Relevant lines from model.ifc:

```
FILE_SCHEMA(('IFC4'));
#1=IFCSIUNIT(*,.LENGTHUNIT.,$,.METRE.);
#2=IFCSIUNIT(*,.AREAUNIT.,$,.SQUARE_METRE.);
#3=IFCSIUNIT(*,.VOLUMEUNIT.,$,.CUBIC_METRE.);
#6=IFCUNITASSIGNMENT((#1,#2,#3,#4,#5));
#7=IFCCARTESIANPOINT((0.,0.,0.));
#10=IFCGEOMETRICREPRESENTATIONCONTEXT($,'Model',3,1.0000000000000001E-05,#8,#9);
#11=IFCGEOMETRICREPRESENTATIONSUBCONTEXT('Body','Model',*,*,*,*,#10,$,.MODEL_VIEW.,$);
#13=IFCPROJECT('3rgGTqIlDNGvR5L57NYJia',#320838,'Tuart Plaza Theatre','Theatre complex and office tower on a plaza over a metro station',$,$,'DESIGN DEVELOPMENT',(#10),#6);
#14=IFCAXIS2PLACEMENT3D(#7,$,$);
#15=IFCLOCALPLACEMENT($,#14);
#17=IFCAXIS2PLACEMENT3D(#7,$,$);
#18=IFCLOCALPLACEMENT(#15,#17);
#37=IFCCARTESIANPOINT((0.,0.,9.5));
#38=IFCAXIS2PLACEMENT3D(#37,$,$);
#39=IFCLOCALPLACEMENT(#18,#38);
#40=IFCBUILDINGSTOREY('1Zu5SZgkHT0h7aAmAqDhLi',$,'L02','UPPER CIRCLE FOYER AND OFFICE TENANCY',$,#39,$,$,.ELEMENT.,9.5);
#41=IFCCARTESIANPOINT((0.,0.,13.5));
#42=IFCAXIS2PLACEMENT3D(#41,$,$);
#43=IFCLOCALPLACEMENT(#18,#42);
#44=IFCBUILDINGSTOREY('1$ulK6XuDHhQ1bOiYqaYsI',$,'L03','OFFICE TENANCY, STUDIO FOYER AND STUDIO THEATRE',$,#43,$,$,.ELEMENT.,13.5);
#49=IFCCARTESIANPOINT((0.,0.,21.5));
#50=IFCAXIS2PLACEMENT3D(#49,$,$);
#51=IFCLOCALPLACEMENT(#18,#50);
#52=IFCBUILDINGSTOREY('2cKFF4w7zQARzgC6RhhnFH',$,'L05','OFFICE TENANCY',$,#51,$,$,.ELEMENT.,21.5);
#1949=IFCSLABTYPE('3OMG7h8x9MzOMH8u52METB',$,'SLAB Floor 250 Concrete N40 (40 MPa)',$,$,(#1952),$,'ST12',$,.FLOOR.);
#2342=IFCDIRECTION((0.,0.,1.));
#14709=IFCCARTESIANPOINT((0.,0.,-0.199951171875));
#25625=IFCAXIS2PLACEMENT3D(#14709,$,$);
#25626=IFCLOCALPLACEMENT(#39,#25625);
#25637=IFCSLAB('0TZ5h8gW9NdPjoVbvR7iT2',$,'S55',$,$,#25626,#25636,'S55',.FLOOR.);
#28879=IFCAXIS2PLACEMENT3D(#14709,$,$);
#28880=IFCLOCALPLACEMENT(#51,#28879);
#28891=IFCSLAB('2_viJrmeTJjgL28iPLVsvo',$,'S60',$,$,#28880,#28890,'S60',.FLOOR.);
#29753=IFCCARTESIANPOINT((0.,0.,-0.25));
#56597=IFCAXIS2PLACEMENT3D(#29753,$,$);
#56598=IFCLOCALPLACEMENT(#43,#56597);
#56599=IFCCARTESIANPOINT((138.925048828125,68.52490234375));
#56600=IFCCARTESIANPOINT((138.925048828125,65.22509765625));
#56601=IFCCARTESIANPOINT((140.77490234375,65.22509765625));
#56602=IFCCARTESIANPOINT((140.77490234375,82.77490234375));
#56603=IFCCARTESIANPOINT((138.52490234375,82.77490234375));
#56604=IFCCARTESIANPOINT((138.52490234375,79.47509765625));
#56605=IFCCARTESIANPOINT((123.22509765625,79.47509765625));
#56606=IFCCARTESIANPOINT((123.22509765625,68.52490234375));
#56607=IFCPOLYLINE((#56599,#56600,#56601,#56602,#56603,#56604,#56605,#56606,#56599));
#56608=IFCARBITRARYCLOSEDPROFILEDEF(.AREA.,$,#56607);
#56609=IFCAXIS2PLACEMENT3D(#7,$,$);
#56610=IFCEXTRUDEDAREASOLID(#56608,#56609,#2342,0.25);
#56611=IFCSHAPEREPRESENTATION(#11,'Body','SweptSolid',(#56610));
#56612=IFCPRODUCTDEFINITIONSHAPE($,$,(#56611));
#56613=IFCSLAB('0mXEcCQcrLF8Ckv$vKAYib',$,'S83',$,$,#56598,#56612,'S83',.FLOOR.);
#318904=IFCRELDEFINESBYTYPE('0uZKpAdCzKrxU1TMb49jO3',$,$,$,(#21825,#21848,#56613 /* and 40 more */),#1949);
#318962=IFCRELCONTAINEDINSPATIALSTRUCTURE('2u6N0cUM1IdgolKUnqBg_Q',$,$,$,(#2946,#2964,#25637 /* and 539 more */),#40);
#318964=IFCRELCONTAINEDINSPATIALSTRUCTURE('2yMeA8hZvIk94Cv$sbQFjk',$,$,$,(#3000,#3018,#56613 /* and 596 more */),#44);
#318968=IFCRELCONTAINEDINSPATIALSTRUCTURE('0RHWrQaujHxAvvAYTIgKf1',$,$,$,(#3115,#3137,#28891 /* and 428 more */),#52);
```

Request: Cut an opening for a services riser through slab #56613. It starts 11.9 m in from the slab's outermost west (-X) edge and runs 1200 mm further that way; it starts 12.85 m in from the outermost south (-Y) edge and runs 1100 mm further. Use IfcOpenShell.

```python
import numpy as np
import ifcopenshell
import ifcopenshell.api.feature
import ifcopenshell.api.geometry
import ifcopenshell.api.root
import ifcopenshell.geom
import ifcopenshell.util.placement
import ifcopenshell.util.representation
import ifcopenshell.util.shape
import ifcopenshell.util.unit

model = ifcopenshell.open("model.ifc")
unit_scale = ifcopenshell.util.unit.calculate_unit_scale(model)
settings = ifcopenshell.geom.settings()


def volume(element):
    """Net volume in cubic metres, openings subtracted."""
    shape = ifcopenshell.geom.create_shape(settings, element)
    return ifcopenshell.util.shape.get_volume(shape.geometry)


slab = model.by_guid("0mXEcCQcrLF8Ckv$vKAYib")
before = volume(slab)

# Extent in the slab's own axes, in metres. The edges named are its -X and -Y sides.
slab_shape = ifcopenshell.geom.create_shape(settings, slab)
vertices = ifcopenshell.util.shape.get_vertices(slab_shape.geometry)
x_min, y_min, bottom = vertices.min(axis=0)
top = vertices[:, 2].max()

opening = ifcopenshell.api.root.create_entity(model, ifc_class="IfcOpeningElement", name="Services riser opening", predefined_type="OPENING")
context = ifcopenshell.util.representation.get_context(model, "Model", "Body", "MODEL_VIEW")
width, depth = 1.2, 1.1
outline = [(0.0, 0.0), (width, 0.0), (width, depth), (0.0, depth), (0.0, 0.0)]
# Overshoot both faces by 50 mm so the cut is clean.
shape = ifcopenshell.api.geometry.add_slab_representation(
    model, context=context, depth=top - bottom + 0.1, polyline=outline
)
ifcopenshell.api.geometry.assign_representation(model, product=opening, representation=shape)

matrix = ifcopenshell.util.placement.get_local_placement(slab.ObjectPlacement)
matrix[:, 3] = matrix @ np.append(np.array([x_min + 11.9, y_min + 12.85, bottom - 0.05]) / unit_scale, 1.0)
ifcopenshell.api.geometry.edit_object_placement(model, product=opening, matrix=matrix, is_si=False)
ifcopenshell.api.feature.add_feature(model, feature=opening, element=slab)

after = volume(slab)

print(f"slab volume {before:.3f} -> {after:.3f} m3")

model.write("model_v2.ifc")
```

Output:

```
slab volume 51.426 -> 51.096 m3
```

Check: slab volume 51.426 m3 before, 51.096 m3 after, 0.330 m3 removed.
